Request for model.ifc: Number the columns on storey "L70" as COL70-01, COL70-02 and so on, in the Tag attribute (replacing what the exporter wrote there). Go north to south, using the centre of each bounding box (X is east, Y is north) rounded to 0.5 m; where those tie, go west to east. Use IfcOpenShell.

First a look at what the model holds.

```python
import ifcopenshell
import ifcopenshell.util.element
import ifcopenshell.util.placement

model = ifcopenshell.open("model.ifc")
print(model.schema)
storey = next(s for s in model.by_type("IfcBuildingStorey") if s.Name == "L70")
columns = [e for e in ifcopenshell.util.element.get_decomposition(storey) if e.is_a("IfcColumn")]
for e in sorted(columns, key=lambda e: e.id()):
    origin = ifcopenshell.util.placement.get_local_placement(e.ObjectPlacement)[:3, 3]
    print(e.id(), e.Tag, e.Name, origin.round(2) + 0.0, sep=" | ")
```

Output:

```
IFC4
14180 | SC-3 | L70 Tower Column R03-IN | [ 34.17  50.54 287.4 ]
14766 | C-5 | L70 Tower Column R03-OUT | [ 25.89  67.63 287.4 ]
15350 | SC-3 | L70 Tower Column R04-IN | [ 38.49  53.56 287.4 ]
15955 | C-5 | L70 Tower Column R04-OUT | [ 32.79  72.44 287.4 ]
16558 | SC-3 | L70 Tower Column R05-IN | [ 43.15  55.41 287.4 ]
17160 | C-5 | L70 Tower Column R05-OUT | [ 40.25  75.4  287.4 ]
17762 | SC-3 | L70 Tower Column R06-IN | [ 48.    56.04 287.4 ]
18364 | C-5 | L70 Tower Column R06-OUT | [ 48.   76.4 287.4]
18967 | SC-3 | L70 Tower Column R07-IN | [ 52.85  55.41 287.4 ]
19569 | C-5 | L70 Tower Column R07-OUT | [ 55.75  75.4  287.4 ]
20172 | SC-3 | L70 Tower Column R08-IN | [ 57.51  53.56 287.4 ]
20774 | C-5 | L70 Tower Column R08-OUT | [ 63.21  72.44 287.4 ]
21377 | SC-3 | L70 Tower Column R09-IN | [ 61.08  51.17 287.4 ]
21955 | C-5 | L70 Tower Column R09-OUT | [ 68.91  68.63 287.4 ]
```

```python
import ifcopenshell
import ifcopenshell.geom
import ifcopenshell.util.element
import ifcopenshell.util.shape

model = ifcopenshell.open("model.ifc")
settings = ifcopenshell.geom.settings()
settings.set("use-world-coords", True)


def centre(element):
    shape = ifcopenshell.geom.create_shape(settings, element)
    return ifcopenshell.util.shape.get_bbox_centroid(shape.geometry)


storey = next(s for s in model.by_type("IfcBuildingStorey") if s.Name == "L70")
columns = [e for e in ifcopenshell.util.element.get_decomposition(storey) if e.is_a("IfcColumn")]

# Insertion points can sit at a corner or the storey origin, so sort by the geometry (in metres).
centres = {e: centre(e) for e in columns}
columns.sort(key=lambda e: (-round(centres[e][1] / 0.5), centres[e][0]))

for i, e in enumerate(columns, start=1):
    number = f"COL70-{i:02d}"
    e.Tag = number
    print(e.id(), number)

model.write("model_v2.ifc")
```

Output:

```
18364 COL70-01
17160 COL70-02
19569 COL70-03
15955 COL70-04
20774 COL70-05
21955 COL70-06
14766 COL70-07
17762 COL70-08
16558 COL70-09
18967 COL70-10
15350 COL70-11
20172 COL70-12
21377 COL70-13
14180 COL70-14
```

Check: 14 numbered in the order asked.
